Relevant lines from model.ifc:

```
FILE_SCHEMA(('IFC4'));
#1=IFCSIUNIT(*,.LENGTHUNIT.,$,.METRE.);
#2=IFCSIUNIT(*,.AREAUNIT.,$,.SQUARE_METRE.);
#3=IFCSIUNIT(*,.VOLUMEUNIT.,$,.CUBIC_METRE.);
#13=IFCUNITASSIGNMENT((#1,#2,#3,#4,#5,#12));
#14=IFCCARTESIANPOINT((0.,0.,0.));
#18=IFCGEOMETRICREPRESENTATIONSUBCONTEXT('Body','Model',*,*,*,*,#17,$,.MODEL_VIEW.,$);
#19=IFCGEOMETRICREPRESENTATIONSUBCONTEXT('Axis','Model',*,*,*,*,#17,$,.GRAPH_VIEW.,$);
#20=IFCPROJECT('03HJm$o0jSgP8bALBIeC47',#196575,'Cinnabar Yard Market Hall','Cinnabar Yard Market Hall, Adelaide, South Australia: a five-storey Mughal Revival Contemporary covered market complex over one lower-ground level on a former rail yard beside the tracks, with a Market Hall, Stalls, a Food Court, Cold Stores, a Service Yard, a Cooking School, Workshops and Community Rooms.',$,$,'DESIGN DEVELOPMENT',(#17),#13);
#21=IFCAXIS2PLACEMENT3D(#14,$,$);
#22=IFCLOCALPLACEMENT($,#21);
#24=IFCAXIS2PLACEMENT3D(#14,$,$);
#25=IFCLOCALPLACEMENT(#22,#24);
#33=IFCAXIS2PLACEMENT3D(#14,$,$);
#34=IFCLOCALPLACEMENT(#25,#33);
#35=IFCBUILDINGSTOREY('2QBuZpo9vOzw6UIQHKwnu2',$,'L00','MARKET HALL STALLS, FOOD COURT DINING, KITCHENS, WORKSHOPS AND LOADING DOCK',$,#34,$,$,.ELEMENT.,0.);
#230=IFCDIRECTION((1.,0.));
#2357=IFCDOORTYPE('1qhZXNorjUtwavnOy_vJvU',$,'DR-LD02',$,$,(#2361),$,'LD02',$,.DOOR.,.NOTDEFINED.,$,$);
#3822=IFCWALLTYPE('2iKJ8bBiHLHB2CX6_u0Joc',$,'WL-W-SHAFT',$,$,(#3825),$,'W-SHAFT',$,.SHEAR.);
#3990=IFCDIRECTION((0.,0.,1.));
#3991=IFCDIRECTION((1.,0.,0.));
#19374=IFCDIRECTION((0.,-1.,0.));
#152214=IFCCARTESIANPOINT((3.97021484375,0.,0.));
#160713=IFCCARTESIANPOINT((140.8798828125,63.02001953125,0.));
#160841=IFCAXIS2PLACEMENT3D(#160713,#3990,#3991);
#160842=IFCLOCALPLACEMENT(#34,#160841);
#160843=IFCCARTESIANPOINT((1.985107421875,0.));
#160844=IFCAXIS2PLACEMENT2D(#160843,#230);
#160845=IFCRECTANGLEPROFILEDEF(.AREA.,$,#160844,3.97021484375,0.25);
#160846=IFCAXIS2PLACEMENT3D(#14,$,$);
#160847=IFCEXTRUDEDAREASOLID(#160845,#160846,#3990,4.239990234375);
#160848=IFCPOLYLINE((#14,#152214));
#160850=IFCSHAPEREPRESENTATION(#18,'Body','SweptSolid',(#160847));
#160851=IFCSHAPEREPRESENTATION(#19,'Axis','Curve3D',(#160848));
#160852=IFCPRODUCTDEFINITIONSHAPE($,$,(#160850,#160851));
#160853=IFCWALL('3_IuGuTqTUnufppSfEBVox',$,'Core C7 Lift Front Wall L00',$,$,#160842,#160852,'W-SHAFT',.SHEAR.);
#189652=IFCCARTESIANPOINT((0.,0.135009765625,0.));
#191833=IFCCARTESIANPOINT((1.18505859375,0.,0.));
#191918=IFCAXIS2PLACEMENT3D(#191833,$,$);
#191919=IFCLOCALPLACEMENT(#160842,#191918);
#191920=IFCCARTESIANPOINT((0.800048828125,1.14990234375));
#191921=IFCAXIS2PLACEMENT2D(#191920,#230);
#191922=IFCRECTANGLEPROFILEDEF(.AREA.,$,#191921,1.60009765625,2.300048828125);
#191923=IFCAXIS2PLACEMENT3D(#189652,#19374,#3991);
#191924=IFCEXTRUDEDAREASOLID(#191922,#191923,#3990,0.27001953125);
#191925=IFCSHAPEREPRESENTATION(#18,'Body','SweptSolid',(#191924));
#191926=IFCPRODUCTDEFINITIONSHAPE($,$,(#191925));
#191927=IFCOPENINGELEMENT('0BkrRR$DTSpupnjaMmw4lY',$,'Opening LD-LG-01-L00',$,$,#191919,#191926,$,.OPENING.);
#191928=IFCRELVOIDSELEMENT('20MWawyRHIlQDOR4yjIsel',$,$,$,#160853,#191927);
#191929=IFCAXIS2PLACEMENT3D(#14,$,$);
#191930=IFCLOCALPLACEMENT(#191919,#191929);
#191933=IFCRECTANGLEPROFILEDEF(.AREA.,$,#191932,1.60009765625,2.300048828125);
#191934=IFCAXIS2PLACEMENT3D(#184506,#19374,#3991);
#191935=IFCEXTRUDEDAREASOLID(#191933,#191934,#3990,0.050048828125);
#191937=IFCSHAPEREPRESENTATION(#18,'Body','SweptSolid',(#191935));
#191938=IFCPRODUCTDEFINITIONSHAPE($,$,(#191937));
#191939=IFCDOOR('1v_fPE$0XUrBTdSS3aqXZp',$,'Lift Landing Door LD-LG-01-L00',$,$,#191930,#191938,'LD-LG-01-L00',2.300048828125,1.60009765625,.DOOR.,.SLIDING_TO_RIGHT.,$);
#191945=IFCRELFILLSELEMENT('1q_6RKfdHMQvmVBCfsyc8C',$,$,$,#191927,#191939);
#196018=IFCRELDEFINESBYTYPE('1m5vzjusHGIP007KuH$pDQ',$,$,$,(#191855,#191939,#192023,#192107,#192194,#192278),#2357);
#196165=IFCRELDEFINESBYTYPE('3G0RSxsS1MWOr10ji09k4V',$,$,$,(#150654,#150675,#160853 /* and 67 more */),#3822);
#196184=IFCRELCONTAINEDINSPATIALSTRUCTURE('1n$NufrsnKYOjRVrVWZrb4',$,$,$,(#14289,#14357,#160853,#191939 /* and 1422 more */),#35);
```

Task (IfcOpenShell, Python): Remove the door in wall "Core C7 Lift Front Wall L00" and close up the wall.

```python
import ifcopenshell
import ifcopenshell.api.feature
import ifcopenshell.api.root
import ifcopenshell.geom
import ifcopenshell.util.shape

model = ifcopenshell.open("model.ifc")
settings = ifcopenshell.geom.settings()


def volume(element):
    """Net volume in cubic metres, openings subtracted."""
    shape = ifcopenshell.geom.create_shape(settings, element)
    return ifcopenshell.util.shape.get_volume(shape.geometry)


door = model.by_id(191939)
opening = door.FillsVoids[0].RelatingOpeningElement
wall = opening.VoidsElements[0].RelatingBuildingElement
before = volume(wall)

ifcopenshell.api.root.remove_product(model, product=door)
ifcopenshell.api.feature.remove_feature(model, feature=opening)

after = volume(wall)

print(f"wall volume {before:.3f} -> {after:.3f} m3")

model.write("model-out.ifc")
```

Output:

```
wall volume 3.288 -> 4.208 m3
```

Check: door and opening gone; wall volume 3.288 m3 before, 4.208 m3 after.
